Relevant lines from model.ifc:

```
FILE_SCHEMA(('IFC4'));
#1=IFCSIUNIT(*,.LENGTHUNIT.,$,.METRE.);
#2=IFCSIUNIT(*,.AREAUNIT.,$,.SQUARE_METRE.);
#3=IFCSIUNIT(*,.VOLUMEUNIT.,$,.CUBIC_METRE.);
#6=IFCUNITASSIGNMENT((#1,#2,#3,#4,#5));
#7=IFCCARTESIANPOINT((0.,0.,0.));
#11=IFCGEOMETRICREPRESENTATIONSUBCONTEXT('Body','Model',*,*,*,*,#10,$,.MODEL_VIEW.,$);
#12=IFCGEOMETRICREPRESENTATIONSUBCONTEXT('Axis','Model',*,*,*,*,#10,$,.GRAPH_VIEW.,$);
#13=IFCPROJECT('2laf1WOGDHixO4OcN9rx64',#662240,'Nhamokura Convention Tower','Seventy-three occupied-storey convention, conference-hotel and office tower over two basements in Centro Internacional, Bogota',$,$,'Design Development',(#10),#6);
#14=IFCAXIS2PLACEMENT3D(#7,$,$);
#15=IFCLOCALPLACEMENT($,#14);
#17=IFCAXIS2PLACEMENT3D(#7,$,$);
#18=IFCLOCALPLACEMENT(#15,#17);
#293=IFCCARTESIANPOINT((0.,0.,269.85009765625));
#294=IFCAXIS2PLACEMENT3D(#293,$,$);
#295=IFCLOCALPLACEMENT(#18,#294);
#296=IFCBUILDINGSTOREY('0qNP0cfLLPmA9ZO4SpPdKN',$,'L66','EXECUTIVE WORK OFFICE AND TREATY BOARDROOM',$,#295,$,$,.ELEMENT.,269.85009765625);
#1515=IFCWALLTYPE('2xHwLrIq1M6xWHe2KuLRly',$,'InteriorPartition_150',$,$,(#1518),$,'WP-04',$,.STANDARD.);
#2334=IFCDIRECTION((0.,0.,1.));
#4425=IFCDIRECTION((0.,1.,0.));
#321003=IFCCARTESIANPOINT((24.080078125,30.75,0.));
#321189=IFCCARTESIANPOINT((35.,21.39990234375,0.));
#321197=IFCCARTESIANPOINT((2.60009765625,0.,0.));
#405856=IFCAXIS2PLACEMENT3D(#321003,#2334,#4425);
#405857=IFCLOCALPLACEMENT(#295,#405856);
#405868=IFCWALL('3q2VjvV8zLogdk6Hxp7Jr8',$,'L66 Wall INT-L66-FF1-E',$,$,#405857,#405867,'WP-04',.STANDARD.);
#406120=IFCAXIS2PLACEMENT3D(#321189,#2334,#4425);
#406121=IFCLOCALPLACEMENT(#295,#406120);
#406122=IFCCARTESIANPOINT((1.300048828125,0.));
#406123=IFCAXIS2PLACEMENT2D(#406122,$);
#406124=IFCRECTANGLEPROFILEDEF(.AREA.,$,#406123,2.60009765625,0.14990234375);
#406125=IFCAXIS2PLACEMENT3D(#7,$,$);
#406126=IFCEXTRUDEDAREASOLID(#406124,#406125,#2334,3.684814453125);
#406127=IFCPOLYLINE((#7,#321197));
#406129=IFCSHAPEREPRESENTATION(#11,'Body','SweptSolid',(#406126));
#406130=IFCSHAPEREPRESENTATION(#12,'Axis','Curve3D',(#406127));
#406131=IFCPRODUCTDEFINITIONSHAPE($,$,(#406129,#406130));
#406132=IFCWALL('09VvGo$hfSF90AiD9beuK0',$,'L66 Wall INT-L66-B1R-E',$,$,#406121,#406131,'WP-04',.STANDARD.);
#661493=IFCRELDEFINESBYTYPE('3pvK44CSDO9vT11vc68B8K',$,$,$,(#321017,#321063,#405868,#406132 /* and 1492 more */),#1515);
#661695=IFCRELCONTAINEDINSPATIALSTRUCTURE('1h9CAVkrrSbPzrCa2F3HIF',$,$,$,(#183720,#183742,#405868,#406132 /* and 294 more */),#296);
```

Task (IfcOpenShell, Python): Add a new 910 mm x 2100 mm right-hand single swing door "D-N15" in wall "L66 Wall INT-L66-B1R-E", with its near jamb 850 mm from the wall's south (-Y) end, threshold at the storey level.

```python
import numpy as np
import ifcopenshell
import ifcopenshell.api.feature
import ifcopenshell.api.geometry
import ifcopenshell.api.root
import ifcopenshell.api.spatial
import ifcopenshell.geom
import ifcopenshell.util.element
import ifcopenshell.util.placement
import ifcopenshell.util.representation
import ifcopenshell.util.shape
import ifcopenshell.util.unit

model = ifcopenshell.open("model.ifc")
unit_scale = ifcopenshell.util.unit.calculate_unit_scale(model)
settings = ifcopenshell.geom.settings()


def volume(element):
    """Net volume in cubic metres, openings subtracted."""
    shape = ifcopenshell.geom.create_shape(settings, element)
    return ifcopenshell.util.shape.get_volume(shape.geometry)


wall = model.by_guid("09VvGo$hfSF90AiD9beuK0")
storey = ifcopenshell.util.element.get_container(wall, ifc_class="IfcBuildingStorey")
context = ifcopenshell.util.representation.get_context(model, "Model", "Body", "MODEL_VIEW")
before = volume(wall)

width, height, from_end, sill = 0.91, 2.1, 0.85, 0.0  # metres

# The wall runs along its own X axis, and the end named is its -X end.
wall_shape = ifcopenshell.geom.create_shape(settings, wall)
x, y, z = ifcopenshell.util.shape.get_vertices(wall_shape.geometry).T
start = x.min() + from_end
face, thickness = float(y.min()), float(y.max() - y.min())
wall_matrix = ifcopenshell.util.placement.get_local_placement(wall.ObjectPlacement)
level = ifcopenshell.util.placement.get_local_placement(storey.ObjectPlacement)[2, 3]


def in_wall(x, y):
    """Placement at x, y metres in the wall's axes, at sill height."""
    matrix = wall_matrix.copy()
    matrix[:, 3] = wall_matrix @ np.array([x / unit_scale, y / unit_scale, 0.0, 1.0])
    matrix[2, 3] = level + sill / unit_scale
    return matrix


# Opening: a box that overshoots both wall faces by 50 mm.
opening = ifcopenshell.api.root.create_entity(model, ifc_class="IfcOpeningElement", predefined_type="OPENING")
box = ifcopenshell.api.geometry.add_wall_representation(
    model, context=context, length=width, height=height, thickness=thickness + 0.1
)
ifcopenshell.api.geometry.assign_representation(model, product=opening, representation=box)
ifcopenshell.api.geometry.edit_object_placement(model, product=opening, matrix=in_wall(start, face - 0.05), is_si=False)
ifcopenshell.api.feature.add_feature(model, feature=opening, element=wall)

door = ifcopenshell.api.root.create_entity(model, ifc_class="IfcDoor", name="D-N15", predefined_type="DOOR")
door.OverallWidth, door.OverallHeight = width / unit_scale, height / unit_scale
door.OperationType = "SINGLE_SWING_RIGHT"
body = ifcopenshell.api.geometry.add_door_representation(
    model,
    context=context,
    overall_width=door.OverallWidth,
    overall_height=door.OverallHeight,
    operation_type="SINGLE_SWING_RIGHT",
    lining_properties={"LiningDepth": thickness / unit_scale, "ThresholdDepth": thickness / unit_scale},
)
ifcopenshell.api.geometry.assign_representation(model, product=door, representation=body)
ifcopenshell.api.spatial.assign_container(model, products=[door], relating_structure=storey)
ifcopenshell.api.feature.add_filling(model, opening=opening, element=door)

# The lining spans the wall, so the door starts at the wall face.
ifcopenshell.api.geometry.edit_object_placement(model, product=door, matrix=in_wall(start, face), is_si=False)

after = volume(wall)

print(f"wall volume {before:.3f} -> {after:.3f} m3")

model.write("model_edited.ifc")
```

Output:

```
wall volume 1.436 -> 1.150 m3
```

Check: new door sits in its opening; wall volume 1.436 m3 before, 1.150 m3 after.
